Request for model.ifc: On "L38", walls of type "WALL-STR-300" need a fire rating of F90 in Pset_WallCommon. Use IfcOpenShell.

First a look at what the model holds.

```python
import ifcopenshell
import ifcopenshell.util.element

model = ifcopenshell.open("model.ifc")
print(model.schema)
storey = next(s for s in model.by_type("IfcBuildingStorey") if s.Name == "L38")
walls = [e for e in ifcopenshell.util.element.get_decomposition(storey) if e.is_a("IfcWall")]
seen = {}
for e in walls:
    element_type = ifcopenshell.util.element.get_type(e)
    key = (element_type.Name if element_type != e and element_type else None, ifcopenshell.util.element.get_pset(e, "Pset_WallCommon", "FireRating"))
    seen[key] = seen.get(key, 0) + 1
for (name, value), count in sorted(seen.items(), key=str):
    print(count, "x", name, "|", value)
```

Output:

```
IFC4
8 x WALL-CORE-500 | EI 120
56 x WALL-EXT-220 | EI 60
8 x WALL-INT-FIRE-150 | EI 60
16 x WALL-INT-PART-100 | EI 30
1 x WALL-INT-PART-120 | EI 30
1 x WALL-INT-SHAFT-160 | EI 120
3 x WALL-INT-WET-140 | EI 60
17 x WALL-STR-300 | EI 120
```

```python
import ifcopenshell
import ifcopenshell.api.pset
import ifcopenshell.util.element

model = ifcopenshell.open("model.ifc")

storey = next(s for s in model.by_type("IfcBuildingStorey") if s.Name == "L38")
walls = [e for e in ifcopenshell.util.element.get_decomposition(storey) if e.is_a("IfcWall")]

count = 0
for e in walls:
    element_type = ifcopenshell.util.element.get_type(e)
    if element_type in (None, e) or element_type.Name != "WALL-STR-300":
        continue
    found = ifcopenshell.util.element.get_pset(e, "Pset_WallCommon", should_inherit=False)
    if found:
        pset = model.by_id(found["id"])
        if len(ifcopenshell.util.element.get_elements_by_pset(pset)) > 1:
            pset = ifcopenshell.api.pset.unshare_pset(model, products=[e], pset=pset)[0]
    else:
        pset = ifcopenshell.api.pset.add_pset(model, product=e, name="Pset_WallCommon")
    ifcopenshell.api.pset.edit_pset(model, pset=pset, properties={"FireRating": "F90"})
    count += 1

print(count, "walls updated")

model.write("model_v2.ifc")
```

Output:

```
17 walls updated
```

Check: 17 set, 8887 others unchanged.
